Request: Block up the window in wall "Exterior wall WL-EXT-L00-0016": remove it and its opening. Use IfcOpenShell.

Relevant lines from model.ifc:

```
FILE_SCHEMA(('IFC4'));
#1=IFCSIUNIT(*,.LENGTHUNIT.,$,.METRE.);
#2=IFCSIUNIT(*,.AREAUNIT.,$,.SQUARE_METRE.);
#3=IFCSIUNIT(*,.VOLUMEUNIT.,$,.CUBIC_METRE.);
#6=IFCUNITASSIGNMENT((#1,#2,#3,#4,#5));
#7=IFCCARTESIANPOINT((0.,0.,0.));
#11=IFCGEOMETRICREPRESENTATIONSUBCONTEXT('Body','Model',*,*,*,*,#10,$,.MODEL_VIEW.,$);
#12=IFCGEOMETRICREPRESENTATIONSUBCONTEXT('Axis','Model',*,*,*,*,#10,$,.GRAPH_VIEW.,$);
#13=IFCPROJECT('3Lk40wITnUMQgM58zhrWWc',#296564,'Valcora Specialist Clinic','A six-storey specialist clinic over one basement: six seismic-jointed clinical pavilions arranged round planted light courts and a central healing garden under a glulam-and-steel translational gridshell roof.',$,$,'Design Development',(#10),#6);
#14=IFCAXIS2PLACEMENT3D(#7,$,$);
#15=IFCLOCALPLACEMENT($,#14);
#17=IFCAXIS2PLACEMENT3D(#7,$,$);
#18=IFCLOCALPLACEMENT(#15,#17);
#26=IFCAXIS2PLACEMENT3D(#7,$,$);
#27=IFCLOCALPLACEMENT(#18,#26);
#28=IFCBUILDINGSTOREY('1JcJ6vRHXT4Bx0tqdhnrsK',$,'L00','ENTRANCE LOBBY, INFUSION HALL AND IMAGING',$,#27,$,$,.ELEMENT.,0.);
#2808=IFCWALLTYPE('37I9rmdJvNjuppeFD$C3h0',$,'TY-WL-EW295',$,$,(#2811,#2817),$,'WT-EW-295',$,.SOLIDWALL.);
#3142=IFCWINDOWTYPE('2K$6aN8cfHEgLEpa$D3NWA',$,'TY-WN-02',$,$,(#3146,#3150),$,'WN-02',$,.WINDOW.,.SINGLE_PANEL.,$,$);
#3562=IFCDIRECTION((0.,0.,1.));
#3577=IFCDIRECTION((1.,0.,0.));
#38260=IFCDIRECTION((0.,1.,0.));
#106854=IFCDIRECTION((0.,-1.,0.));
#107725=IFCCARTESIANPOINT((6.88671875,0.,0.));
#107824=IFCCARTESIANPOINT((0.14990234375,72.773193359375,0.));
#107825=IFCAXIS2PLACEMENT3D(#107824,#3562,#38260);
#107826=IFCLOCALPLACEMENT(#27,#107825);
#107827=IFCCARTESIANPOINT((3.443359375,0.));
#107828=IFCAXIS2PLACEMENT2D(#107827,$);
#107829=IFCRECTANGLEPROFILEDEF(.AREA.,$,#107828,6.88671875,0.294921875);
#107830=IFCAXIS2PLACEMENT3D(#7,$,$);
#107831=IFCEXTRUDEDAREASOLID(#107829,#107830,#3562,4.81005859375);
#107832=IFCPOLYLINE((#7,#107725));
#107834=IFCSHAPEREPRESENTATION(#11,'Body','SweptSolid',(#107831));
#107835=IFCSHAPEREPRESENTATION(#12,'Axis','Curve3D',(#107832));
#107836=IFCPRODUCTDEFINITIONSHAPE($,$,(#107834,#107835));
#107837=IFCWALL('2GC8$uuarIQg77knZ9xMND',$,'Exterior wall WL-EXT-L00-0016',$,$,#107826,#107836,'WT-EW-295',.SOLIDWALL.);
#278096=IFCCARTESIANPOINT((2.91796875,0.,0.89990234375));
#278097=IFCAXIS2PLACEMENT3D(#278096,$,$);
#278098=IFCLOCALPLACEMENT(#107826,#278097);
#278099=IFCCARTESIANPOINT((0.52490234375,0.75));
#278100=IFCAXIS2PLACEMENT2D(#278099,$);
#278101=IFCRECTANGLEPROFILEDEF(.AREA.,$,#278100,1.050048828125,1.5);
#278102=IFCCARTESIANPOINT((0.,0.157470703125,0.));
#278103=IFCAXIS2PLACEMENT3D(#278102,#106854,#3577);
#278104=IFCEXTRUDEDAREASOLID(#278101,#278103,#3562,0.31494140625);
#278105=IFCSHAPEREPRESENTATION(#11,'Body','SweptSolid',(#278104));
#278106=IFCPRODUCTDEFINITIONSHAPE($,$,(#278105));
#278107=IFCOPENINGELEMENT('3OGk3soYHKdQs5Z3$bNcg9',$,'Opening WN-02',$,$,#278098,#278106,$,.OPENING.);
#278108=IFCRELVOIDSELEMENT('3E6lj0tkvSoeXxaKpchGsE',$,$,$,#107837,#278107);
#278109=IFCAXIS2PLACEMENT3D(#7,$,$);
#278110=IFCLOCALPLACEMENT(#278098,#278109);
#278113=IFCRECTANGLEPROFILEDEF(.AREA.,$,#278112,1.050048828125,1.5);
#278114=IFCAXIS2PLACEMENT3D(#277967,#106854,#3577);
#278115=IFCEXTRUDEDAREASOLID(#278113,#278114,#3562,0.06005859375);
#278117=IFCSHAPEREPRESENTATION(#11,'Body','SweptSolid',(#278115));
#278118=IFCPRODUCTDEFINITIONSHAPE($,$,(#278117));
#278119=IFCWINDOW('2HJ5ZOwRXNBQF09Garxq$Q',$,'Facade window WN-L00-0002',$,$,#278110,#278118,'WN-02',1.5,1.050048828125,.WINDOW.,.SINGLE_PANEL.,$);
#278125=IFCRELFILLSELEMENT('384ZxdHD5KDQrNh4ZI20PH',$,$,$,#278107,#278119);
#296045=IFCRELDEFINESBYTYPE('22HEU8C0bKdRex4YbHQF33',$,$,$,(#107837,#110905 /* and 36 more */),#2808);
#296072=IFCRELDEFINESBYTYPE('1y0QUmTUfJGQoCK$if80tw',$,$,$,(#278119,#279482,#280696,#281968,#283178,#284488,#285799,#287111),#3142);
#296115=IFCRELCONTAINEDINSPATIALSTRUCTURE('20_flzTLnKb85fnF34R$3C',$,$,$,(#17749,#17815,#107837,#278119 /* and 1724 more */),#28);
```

```python
import ifcopenshell
import ifcopenshell.api.feature
import ifcopenshell.api.root
import ifcopenshell.geom
import ifcopenshell.util.shape

model = ifcopenshell.open("model.ifc")
settings = ifcopenshell.geom.settings()


def volume(element):
    """Net volume in cubic metres, openings subtracted."""
    shape = ifcopenshell.geom.create_shape(settings, element)
    return ifcopenshell.util.shape.get_volume(shape.geometry)


window = model.by_guid("2HJ5ZOwRXNBQF09Garxq$Q")
opening = window.FillsVoids[0].RelatingOpeningElement
wall = opening.VoidsElements[0].RelatingBuildingElement
before = volume(wall)

ifcopenshell.api.root.remove_product(model, product=window)
ifcopenshell.api.feature.remove_feature(model, feature=opening)

after = volume(wall)

print(f"wall volume {before:.3f} -> {after:.3f} m3")

model.write("model_edited.ifc")
```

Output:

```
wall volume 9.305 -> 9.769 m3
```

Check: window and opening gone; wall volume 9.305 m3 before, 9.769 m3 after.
